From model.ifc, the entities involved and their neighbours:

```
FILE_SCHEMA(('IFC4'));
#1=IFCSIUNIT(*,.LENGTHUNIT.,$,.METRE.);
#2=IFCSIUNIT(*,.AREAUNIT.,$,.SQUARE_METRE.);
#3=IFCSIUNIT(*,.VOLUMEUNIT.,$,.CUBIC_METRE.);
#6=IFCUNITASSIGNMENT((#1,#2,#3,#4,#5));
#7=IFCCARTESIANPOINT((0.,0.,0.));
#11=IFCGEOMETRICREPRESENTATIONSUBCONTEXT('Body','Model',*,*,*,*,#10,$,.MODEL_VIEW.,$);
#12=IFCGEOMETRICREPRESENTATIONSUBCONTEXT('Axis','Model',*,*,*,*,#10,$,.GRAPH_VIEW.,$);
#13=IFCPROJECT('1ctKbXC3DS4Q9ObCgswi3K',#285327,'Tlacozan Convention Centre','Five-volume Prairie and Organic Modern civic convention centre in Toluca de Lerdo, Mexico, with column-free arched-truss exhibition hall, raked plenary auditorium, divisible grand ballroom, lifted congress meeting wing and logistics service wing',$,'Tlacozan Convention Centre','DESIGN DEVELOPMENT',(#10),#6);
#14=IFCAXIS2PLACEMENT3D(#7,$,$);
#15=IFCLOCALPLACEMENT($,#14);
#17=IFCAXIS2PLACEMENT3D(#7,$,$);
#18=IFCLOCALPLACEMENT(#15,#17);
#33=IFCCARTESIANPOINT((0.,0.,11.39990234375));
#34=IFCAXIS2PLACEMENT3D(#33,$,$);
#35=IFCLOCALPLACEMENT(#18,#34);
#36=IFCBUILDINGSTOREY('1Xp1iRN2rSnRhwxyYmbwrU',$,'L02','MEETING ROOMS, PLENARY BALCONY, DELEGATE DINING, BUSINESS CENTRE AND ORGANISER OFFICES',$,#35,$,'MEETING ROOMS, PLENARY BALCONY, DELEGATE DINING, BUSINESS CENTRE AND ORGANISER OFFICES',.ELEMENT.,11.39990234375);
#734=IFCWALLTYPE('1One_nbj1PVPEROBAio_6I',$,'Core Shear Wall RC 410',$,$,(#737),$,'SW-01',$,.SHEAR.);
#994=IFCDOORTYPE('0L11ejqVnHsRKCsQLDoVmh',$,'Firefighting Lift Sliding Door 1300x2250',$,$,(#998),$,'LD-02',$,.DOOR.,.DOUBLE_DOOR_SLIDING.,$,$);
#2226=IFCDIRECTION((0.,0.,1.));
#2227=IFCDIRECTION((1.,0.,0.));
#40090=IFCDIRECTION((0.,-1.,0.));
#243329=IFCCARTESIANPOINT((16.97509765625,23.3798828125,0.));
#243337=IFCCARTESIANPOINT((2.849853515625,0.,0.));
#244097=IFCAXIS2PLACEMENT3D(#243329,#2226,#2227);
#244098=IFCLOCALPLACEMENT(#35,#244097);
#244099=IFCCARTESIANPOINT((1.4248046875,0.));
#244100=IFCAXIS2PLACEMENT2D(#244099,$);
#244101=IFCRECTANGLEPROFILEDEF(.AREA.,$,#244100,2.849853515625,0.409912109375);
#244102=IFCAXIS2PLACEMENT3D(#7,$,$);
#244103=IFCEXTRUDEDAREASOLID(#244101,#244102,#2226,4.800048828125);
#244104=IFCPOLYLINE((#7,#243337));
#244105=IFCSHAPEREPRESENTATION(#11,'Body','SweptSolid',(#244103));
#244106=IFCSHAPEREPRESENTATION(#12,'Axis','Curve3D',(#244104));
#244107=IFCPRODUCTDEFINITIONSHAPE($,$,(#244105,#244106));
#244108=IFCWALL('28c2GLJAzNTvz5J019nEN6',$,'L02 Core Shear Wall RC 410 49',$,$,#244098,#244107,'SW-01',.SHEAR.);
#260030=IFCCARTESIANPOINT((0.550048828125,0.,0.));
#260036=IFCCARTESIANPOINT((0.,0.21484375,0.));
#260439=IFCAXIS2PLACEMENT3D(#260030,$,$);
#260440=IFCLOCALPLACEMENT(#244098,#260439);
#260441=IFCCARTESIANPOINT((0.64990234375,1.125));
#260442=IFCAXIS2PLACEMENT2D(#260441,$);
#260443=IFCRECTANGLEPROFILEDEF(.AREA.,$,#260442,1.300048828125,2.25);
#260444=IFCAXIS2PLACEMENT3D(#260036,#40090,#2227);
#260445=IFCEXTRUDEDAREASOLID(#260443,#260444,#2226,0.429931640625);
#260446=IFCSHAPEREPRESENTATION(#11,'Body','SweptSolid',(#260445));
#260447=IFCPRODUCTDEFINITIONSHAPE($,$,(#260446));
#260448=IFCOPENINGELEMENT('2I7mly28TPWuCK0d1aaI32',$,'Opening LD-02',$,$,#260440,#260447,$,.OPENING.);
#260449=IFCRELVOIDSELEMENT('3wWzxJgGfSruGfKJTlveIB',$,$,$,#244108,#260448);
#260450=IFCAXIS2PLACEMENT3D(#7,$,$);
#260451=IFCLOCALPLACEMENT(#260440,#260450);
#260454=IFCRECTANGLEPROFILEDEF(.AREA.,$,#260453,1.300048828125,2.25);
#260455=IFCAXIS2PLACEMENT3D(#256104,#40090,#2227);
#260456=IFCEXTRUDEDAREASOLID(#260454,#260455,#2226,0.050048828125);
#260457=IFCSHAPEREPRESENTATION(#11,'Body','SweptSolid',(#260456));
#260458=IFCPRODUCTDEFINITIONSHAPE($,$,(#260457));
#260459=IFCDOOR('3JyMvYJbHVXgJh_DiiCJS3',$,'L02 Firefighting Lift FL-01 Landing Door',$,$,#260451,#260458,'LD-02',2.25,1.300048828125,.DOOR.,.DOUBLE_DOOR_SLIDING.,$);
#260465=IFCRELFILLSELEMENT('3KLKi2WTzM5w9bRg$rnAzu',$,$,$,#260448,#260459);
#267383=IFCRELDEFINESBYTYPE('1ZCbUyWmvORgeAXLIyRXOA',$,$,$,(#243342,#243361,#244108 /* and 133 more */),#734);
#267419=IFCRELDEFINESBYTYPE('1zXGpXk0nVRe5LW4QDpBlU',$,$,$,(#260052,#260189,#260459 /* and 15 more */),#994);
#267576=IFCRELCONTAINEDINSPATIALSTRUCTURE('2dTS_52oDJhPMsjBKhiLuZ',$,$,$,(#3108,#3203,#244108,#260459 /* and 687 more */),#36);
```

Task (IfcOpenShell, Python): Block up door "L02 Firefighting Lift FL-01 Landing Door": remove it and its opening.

```python
import ifcopenshell
import ifcopenshell.api.feature
import ifcopenshell.api.root
import ifcopenshell.geom
import ifcopenshell.util.shape

model = ifcopenshell.open("model.ifc")
settings = ifcopenshell.geom.settings()


def volume(element):
    """Net volume in cubic metres, openings subtracted."""
    shape = ifcopenshell.geom.create_shape(settings, element)
    return ifcopenshell.util.shape.get_volume(shape.geometry)


door = model.by_guid("3JyMvYJbHVXgJh_DiiCJS3")
opening = door.FillsVoids[0].RelatingOpeningElement
wall = opening.VoidsElements[0].RelatingBuildingElement
before = volume(wall)

ifcopenshell.api.root.remove_product(model, product=door)
ifcopenshell.api.feature.remove_feature(model, feature=opening)

after = volume(wall)

print(f"wall volume {before:.3f} -> {after:.3f} m3")

model.write("model_edited.ifc")
```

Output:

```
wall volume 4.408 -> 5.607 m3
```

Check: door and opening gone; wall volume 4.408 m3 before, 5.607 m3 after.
